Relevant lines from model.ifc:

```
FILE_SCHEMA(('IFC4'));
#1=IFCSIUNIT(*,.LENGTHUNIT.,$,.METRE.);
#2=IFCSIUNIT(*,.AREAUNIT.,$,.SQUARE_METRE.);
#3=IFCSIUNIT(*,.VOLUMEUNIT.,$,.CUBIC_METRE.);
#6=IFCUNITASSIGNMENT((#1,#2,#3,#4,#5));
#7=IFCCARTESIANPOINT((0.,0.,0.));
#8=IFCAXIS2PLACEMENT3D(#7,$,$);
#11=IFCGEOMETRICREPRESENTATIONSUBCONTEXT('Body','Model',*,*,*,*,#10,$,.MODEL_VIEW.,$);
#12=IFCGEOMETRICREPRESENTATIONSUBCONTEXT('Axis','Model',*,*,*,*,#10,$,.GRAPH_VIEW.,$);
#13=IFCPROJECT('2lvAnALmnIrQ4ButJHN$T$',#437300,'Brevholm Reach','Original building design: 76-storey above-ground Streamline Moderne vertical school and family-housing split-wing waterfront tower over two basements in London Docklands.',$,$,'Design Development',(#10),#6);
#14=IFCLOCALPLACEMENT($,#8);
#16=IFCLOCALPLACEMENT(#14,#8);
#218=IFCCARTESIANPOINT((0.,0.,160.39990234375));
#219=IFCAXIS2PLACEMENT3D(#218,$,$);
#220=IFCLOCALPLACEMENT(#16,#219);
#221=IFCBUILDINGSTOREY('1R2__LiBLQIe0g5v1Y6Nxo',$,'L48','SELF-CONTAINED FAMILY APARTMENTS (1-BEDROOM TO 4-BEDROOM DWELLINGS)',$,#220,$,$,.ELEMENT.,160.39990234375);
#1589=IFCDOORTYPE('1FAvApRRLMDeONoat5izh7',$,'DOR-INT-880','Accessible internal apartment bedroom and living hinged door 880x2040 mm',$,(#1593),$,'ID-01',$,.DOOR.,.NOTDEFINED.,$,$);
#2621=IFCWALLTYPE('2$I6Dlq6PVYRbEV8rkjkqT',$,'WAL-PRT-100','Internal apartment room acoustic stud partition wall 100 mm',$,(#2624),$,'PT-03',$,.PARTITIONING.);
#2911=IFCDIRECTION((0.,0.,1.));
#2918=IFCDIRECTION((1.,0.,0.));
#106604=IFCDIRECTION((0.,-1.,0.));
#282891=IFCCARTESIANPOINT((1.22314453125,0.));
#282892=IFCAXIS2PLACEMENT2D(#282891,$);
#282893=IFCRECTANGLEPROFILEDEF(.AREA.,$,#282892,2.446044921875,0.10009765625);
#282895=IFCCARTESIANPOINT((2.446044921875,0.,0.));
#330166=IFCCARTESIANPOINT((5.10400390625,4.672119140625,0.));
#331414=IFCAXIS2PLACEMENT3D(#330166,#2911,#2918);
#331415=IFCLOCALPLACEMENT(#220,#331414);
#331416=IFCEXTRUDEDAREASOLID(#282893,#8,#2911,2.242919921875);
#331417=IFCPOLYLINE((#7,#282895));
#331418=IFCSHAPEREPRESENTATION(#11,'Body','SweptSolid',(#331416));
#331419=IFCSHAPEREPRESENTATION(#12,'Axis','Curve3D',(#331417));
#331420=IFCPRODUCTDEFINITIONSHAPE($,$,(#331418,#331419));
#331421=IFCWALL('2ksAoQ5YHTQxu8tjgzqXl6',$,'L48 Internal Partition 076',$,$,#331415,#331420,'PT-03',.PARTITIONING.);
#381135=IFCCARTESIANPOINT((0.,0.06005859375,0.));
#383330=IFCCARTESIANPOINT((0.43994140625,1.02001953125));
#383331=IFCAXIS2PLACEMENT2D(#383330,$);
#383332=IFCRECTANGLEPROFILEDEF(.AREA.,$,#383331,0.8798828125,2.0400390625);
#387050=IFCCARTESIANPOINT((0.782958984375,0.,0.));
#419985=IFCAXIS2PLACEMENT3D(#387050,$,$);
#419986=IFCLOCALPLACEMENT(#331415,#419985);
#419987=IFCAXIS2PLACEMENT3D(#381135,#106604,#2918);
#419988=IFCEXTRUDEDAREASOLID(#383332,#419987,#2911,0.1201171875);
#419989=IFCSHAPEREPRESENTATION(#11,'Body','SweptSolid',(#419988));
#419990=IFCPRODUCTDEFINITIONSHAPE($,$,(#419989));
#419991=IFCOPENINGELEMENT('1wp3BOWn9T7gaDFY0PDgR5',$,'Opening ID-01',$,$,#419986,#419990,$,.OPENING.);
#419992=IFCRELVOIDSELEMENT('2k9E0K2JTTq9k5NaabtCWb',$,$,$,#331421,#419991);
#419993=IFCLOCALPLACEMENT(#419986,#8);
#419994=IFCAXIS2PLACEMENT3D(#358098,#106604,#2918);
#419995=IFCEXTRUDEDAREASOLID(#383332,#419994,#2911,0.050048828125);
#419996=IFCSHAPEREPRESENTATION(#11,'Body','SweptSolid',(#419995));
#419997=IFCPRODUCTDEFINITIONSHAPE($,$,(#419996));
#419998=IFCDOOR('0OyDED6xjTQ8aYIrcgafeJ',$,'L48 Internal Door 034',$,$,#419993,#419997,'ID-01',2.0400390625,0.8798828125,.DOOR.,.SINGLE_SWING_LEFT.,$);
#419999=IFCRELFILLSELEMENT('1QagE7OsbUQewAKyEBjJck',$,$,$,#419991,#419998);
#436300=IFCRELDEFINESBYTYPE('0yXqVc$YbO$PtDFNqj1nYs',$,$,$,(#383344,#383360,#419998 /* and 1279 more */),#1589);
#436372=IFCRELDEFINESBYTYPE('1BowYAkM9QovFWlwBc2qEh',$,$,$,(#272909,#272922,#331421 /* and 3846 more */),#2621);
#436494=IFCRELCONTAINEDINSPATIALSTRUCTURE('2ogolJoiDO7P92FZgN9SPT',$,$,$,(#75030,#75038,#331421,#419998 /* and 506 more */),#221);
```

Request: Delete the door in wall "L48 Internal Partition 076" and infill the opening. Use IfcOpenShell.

```python
import ifcopenshell
import ifcopenshell.api.feature
import ifcopenshell.api.root
import ifcopenshell.geom
import ifcopenshell.util.shape

model = ifcopenshell.open("model.ifc")
settings = ifcopenshell.geom.settings()


def volume(element):
    """Net volume in cubic metres, openings subtracted."""
    shape = ifcopenshell.geom.create_shape(settings, element)
    return ifcopenshell.util.shape.get_volume(shape.geometry)


door = model.by_guid("0OyDED6xjTQ8aYIrcgafeJ")
opening = door.FillsVoids[0].RelatingOpeningElement
wall = opening.VoidsElements[0].RelatingBuildingElement
before = volume(wall)

ifcopenshell.api.root.remove_product(model, product=door)
ifcopenshell.api.feature.remove_feature(model, feature=opening)

after = volume(wall)

print(f"wall volume {before:.3f} -> {after:.3f} m3")

model.write("model-out.ifc")
```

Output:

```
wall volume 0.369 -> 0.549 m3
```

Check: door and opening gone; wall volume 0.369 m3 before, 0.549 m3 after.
